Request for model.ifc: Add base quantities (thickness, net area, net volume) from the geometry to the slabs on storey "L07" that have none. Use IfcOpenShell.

First a look at what the model holds.

```python
import ifcopenshell
import ifcopenshell.util.element
import ifcopenshell.util.unit

model = ifcopenshell.open("model.ifc")
print(model.schema)
for unit_type in ("LENGTHUNIT", "AREAUNIT", "VOLUMEUNIT"):
    print(unit_type, ifcopenshell.util.unit.calculate_unit_scale(model, unit_type))
storey = next(s for s in model.by_type("IfcBuildingStorey") if s.Name == "L07")
slabs = [e for e in ifcopenshell.util.element.get_decomposition(storey) if e.is_a("IfcSlab")]
for e in sorted(slabs, key=lambda e: e.id()):
    print(e.id(), e.is_a(), e.Name, list(ifcopenshell.util.element.get_psets(e, qtos_only=True)), sep=" | ")
```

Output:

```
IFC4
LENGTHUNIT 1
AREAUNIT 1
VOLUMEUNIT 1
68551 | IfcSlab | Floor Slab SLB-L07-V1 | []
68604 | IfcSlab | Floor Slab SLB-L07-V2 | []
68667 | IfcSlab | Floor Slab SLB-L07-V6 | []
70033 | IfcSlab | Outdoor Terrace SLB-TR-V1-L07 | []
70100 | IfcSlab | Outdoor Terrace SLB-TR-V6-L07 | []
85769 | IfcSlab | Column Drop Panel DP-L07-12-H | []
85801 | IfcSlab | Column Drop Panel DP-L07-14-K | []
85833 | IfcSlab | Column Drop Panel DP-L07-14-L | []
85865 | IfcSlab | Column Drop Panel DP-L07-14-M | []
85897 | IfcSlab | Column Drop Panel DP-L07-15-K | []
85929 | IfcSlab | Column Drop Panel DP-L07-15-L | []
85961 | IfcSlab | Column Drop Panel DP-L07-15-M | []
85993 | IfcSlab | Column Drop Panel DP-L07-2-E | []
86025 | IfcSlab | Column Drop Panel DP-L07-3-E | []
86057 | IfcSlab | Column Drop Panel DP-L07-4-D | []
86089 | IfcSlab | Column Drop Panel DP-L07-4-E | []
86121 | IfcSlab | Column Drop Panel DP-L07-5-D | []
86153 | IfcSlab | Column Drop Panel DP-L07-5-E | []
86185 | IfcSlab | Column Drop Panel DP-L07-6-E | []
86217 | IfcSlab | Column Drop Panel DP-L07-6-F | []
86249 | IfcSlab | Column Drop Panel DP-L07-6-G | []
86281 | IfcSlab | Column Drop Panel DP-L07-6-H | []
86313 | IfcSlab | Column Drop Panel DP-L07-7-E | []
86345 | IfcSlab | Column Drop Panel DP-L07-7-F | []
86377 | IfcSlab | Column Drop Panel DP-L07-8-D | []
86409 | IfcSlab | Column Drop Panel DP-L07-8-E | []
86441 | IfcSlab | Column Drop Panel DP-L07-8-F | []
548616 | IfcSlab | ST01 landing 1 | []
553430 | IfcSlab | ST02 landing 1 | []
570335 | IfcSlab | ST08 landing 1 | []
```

```python
import ifcopenshell
import ifcopenshell.api.pset
import ifcopenshell.geom
import ifcopenshell.util.element
import ifcopenshell.util.shape
import ifcopenshell.util.unit

model = ifcopenshell.open("model.ifc")
unit_scale = ifcopenshell.util.unit.calculate_unit_scale(model)
area_scale = ifcopenshell.util.unit.calculate_unit_scale(model, "AREAUNIT")
volume_scale = ifcopenshell.util.unit.calculate_unit_scale(model, "VOLUMEUNIT")
settings = ifcopenshell.geom.settings()

storey = next(s for s in model.by_type("IfcBuildingStorey") if s.Name == "L07")
slabs = [e for e in ifcopenshell.util.element.get_decomposition(storey) if e.is_a("IfcSlab")]

for e in sorted(slabs, key=lambda e: e.id()):
    if ifcopenshell.util.element.get_psets(e, qtos_only=True, should_inherit=False):
        continue
    # Geometry comes back in metres, in the element's own axes.
    shape = ifcopenshell.geom.create_shape(settings, e)
    values = {
        "Width": ifcopenshell.util.shape.get_z(shape.geometry) / unit_scale,
        "NetArea": ifcopenshell.util.shape.get_footprint_area(shape.geometry) / area_scale,
        "NetVolume": ifcopenshell.util.shape.get_volume(shape.geometry) / volume_scale,
    }
    qto = ifcopenshell.api.pset.add_qto(model, product=e, name="Qto_SlabBaseQuantities")
    ifcopenshell.api.pset.edit_qto(model, qto=qto, properties=values)
    print(e.id(), {k: round(v, 3) for k, v in values.items()})

model.write("model_rev.ifc")
```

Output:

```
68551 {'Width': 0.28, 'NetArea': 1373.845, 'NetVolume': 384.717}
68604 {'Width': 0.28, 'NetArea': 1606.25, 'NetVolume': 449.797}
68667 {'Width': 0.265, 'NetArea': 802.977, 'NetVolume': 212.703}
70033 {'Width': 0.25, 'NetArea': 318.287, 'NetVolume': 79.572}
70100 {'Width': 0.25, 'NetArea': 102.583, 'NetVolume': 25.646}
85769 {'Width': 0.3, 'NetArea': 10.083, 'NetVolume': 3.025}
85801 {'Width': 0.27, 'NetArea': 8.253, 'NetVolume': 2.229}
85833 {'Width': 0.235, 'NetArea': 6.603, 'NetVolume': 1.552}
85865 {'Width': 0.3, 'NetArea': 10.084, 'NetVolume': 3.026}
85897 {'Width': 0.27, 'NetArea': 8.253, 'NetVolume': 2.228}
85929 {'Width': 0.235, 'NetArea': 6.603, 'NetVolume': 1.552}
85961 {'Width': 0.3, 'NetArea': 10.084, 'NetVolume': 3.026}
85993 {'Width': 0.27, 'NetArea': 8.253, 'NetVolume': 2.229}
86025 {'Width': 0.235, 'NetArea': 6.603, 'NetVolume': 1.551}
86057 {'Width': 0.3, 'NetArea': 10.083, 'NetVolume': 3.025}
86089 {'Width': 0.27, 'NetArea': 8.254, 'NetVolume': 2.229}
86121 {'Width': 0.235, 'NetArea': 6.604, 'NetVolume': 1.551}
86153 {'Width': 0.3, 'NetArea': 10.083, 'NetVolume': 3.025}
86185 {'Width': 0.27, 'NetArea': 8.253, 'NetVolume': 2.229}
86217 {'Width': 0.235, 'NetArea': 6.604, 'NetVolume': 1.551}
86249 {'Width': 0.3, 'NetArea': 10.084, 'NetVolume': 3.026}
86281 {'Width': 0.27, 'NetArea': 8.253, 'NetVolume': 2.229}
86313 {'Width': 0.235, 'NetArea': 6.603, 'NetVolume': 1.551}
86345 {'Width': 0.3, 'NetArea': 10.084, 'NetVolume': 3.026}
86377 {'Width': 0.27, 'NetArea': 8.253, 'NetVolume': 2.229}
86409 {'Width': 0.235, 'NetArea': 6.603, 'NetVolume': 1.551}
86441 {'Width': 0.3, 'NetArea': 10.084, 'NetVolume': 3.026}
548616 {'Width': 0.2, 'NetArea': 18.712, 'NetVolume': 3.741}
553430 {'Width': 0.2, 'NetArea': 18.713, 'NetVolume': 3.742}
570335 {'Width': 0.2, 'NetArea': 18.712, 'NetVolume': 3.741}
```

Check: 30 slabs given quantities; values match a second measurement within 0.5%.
